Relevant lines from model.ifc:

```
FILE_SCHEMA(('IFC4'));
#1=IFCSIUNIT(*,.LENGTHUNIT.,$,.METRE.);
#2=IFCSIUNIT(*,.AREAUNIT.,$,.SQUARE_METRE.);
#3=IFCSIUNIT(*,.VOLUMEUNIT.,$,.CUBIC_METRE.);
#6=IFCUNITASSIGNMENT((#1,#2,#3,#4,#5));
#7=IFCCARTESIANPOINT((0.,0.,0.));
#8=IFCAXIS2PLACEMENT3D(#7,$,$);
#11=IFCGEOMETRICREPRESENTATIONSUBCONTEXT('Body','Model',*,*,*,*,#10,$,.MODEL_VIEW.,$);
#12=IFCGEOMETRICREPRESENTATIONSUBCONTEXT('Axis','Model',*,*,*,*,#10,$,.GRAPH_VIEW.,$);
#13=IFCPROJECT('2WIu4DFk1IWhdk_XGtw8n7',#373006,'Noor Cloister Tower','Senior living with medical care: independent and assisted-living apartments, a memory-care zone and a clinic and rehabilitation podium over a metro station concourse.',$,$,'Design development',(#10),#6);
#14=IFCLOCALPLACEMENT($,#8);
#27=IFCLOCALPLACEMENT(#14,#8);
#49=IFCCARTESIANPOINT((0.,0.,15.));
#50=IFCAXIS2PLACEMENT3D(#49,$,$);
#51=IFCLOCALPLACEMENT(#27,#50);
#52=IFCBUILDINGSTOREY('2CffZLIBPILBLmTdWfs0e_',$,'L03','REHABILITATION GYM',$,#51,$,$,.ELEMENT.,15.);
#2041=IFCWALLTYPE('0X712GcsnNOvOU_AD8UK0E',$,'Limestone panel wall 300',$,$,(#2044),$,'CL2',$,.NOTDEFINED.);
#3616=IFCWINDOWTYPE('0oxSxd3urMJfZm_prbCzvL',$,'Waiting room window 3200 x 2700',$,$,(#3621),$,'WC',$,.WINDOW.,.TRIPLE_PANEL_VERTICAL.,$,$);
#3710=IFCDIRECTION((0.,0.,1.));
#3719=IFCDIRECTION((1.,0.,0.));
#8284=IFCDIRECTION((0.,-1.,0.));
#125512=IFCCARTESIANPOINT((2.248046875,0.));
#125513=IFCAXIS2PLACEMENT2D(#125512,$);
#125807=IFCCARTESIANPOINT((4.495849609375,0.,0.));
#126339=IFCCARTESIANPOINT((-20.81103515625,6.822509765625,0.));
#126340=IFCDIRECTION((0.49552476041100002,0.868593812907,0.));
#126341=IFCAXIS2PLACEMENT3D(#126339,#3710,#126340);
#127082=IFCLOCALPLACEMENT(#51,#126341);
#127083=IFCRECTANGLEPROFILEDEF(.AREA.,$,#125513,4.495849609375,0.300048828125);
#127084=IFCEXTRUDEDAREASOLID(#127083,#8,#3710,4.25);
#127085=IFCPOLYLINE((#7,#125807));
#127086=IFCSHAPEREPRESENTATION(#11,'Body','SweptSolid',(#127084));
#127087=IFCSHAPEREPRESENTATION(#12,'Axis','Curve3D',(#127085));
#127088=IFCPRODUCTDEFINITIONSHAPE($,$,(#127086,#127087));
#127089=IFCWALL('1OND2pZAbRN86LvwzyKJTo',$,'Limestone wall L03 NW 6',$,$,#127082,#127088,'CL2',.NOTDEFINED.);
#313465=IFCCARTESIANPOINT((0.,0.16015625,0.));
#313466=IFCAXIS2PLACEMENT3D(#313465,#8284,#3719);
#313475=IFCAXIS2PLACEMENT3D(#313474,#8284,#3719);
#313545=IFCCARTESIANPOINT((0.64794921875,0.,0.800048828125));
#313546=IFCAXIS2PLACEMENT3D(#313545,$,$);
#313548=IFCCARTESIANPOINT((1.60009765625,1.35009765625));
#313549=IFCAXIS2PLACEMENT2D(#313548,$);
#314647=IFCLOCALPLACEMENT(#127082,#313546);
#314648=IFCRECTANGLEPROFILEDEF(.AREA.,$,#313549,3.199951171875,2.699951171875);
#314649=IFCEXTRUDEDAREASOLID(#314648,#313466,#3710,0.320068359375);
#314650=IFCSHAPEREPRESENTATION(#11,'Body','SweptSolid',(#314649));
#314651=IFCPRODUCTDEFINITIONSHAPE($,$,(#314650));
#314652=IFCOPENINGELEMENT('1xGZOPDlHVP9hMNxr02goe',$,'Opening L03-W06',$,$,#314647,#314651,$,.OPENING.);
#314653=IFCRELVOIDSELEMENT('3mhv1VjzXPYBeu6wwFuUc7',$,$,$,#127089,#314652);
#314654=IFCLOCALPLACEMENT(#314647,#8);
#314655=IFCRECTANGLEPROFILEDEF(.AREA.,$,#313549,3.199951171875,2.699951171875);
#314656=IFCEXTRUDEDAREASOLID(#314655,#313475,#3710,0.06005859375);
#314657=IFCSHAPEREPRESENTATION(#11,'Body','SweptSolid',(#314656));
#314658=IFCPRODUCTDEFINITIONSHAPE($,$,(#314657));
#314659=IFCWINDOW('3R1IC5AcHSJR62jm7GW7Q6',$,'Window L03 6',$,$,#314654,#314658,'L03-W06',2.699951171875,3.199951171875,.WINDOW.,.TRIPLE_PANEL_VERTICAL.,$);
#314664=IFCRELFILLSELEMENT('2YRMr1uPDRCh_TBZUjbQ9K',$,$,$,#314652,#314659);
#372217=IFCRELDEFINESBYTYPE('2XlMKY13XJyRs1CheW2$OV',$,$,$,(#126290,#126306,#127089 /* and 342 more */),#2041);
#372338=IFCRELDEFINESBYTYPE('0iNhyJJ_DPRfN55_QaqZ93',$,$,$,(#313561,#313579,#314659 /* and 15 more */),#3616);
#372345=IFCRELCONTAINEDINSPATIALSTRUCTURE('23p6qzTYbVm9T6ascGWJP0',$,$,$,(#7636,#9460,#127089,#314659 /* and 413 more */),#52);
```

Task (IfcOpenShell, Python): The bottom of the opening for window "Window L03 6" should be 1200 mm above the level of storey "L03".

```python
import numpy as np
import ifcopenshell
import ifcopenshell.api.geometry
import ifcopenshell.geom
import ifcopenshell.util.element
import ifcopenshell.util.placement
import ifcopenshell.util.shape
import ifcopenshell.util.unit

model = ifcopenshell.open("model.ifc")
unit_scale = ifcopenshell.util.unit.calculate_unit_scale(model)

window = model.by_id(314659)
opening = window.FillsVoids[0].RelatingOpeningElement
storey = ifcopenshell.util.element.get_container(window, ifc_class="IfcBuildingStorey")
level = ifcopenshell.util.placement.get_local_placement(storey.ObjectPlacement)[2, 3]

# The opening's origin need not be at the sill, so measure its lowest point.
shape = ifcopenshell.geom.create_shape(ifcopenshell.geom.settings(), opening)
bottom = ifcopenshell.util.shape.get_shape_bottom_elevation(shape, shape.geometry) / unit_scale
dz = level + 1.2 / unit_scale - bottom

shift = np.array([0.0, 0.0, dz])
# The window is placed relative to its opening, so it follows when the opening moves.
matrix = ifcopenshell.util.placement.get_local_placement(opening.ObjectPlacement)
matrix[:3, 3] += shift
ifcopenshell.api.geometry.edit_object_placement(
    model, product=opening, matrix=matrix, is_si=False, should_transform_children=True
)

print(f"moved by {dz * unit_scale:+.3f} m")

model.write("model_edited.ifc")
```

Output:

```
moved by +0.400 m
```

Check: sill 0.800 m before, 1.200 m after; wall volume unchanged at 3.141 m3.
